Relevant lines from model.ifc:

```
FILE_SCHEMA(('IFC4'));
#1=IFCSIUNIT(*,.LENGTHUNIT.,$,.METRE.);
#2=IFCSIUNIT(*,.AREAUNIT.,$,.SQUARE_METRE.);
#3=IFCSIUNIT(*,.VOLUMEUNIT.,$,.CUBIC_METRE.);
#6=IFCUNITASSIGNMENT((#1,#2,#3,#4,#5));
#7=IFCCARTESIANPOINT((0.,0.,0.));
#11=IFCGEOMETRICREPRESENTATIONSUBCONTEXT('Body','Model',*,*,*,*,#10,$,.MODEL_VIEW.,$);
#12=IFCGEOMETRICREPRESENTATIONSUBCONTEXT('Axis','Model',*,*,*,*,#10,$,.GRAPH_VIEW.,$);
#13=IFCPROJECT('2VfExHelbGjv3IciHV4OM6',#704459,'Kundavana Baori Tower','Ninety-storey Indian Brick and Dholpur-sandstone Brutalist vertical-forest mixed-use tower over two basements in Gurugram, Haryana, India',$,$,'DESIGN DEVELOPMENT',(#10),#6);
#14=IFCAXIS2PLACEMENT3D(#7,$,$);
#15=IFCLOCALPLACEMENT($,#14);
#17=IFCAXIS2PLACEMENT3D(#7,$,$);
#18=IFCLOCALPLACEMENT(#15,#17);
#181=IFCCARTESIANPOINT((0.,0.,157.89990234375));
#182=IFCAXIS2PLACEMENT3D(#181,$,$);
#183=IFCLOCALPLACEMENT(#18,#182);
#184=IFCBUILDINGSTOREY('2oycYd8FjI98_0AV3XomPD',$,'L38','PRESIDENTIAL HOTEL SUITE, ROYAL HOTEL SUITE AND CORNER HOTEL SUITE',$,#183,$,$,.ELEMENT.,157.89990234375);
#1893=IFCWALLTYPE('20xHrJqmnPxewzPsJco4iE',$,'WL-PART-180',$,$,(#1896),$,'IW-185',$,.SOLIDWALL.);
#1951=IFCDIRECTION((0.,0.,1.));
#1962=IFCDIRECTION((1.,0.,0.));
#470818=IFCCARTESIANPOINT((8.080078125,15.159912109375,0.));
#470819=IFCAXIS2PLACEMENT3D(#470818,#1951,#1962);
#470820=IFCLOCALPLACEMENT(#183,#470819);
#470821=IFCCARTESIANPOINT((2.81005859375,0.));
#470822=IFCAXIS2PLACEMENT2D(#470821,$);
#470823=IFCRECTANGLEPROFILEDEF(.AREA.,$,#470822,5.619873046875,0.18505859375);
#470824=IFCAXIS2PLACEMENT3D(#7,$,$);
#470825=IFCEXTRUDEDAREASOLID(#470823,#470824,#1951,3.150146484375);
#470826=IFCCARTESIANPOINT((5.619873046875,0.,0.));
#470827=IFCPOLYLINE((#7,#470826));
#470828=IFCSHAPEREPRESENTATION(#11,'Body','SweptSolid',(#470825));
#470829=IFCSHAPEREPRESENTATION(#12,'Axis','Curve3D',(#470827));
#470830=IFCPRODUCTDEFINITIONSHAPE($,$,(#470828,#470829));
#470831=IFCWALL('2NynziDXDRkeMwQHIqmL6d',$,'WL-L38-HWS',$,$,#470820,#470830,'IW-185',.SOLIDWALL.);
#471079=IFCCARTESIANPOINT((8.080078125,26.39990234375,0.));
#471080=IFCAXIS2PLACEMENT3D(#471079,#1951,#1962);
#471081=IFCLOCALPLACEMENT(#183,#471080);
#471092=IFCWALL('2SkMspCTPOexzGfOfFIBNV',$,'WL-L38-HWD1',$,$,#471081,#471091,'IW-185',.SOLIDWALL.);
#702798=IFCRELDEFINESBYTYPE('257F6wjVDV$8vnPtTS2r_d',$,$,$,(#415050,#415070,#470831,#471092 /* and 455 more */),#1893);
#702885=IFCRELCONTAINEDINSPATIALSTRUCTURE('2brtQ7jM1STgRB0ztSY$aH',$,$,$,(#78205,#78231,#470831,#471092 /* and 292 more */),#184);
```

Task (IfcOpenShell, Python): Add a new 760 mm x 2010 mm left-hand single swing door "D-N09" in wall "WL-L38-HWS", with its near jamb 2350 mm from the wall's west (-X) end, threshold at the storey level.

```python
import numpy as np
import ifcopenshell
import ifcopenshell.api.feature
import ifcopenshell.api.geometry
import ifcopenshell.api.root
import ifcopenshell.api.spatial
import ifcopenshell.geom
import ifcopenshell.util.element
import ifcopenshell.util.placement
import ifcopenshell.util.representation
import ifcopenshell.util.shape
import ifcopenshell.util.unit

model = ifcopenshell.open("model.ifc")
unit_scale = ifcopenshell.util.unit.calculate_unit_scale(model)
settings = ifcopenshell.geom.settings()


def volume(element):
    """Net volume in cubic metres, openings subtracted."""
    shape = ifcopenshell.geom.create_shape(settings, element)
    return ifcopenshell.util.shape.get_volume(shape.geometry)


wall = model.by_guid("2NynziDXDRkeMwQHIqmL6d")
storey = ifcopenshell.util.element.get_container(wall, ifc_class="IfcBuildingStorey")
context = ifcopenshell.util.representation.get_context(model, "Model", "Body", "MODEL_VIEW")
before = volume(wall)

width, height, from_end, sill = 0.76, 2.01, 2.35, 0.0  # metres

# The wall runs along its own X axis, and the end named is its -X end.
wall_shape = ifcopenshell.geom.create_shape(settings, wall)
x, y, z = ifcopenshell.util.shape.get_vertices(wall_shape.geometry).T
start = x.min() + from_end
face, thickness = float(y.min()), float(y.max() - y.min())
wall_matrix = ifcopenshell.util.placement.get_local_placement(wall.ObjectPlacement)
level = ifcopenshell.util.placement.get_local_placement(storey.ObjectPlacement)[2, 3]


def in_wall(x, y):
    """Placement at x, y metres in the wall's axes, at sill height."""
    matrix = wall_matrix.copy()
    matrix[:, 3] = wall_matrix @ np.array([x / unit_scale, y / unit_scale, 0.0, 1.0])
    matrix[2, 3] = level + sill / unit_scale
    return matrix


# Opening: a box that overshoots both wall faces by 50 mm.
opening = ifcopenshell.api.root.create_entity(model, ifc_class="IfcOpeningElement", predefined_type="OPENING")
box = ifcopenshell.api.geometry.add_wall_representation(
    model, context=context, length=width, height=height, thickness=thickness + 0.1
)
ifcopenshell.api.geometry.assign_representation(model, product=opening, representation=box)
ifcopenshell.api.geometry.edit_object_placement(model, product=opening, matrix=in_wall(start, face - 0.05), is_si=False)
ifcopenshell.api.feature.add_feature(model, feature=opening, element=wall)

door = ifcopenshell.api.root.create_entity(model, ifc_class="IfcDoor", name="D-N09", predefined_type="DOOR")
door.OverallWidth, door.OverallHeight = width / unit_scale, height / unit_scale
door.OperationType = "SINGLE_SWING_LEFT"
body = ifcopenshell.api.geometry.add_door_representation(
    model,
    context=context,
    overall_width=door.OverallWidth,
    overall_height=door.OverallHeight,
    operation_type="SINGLE_SWING_LEFT",
    lining_properties={"LiningDepth": thickness / unit_scale, "ThresholdDepth": thickness / unit_scale},
)
ifcopenshell.api.geometry.assign_representation(model, product=door, representation=body)
ifcopenshell.api.spatial.assign_container(model, products=[door], relating_structure=storey)
ifcopenshell.api.feature.add_filling(model, opening=opening, element=door)

# The lining spans the wall, so the door starts at the wall face.
ifcopenshell.api.geometry.edit_object_placement(model, product=door, matrix=in_wall(start, face), is_si=False)

after = volume(wall)

print(f"wall volume {before:.3f} -> {after:.3f} m3")

model.write("model_rev.ifc")
```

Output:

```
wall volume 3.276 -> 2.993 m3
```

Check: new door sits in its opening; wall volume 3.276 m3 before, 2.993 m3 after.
